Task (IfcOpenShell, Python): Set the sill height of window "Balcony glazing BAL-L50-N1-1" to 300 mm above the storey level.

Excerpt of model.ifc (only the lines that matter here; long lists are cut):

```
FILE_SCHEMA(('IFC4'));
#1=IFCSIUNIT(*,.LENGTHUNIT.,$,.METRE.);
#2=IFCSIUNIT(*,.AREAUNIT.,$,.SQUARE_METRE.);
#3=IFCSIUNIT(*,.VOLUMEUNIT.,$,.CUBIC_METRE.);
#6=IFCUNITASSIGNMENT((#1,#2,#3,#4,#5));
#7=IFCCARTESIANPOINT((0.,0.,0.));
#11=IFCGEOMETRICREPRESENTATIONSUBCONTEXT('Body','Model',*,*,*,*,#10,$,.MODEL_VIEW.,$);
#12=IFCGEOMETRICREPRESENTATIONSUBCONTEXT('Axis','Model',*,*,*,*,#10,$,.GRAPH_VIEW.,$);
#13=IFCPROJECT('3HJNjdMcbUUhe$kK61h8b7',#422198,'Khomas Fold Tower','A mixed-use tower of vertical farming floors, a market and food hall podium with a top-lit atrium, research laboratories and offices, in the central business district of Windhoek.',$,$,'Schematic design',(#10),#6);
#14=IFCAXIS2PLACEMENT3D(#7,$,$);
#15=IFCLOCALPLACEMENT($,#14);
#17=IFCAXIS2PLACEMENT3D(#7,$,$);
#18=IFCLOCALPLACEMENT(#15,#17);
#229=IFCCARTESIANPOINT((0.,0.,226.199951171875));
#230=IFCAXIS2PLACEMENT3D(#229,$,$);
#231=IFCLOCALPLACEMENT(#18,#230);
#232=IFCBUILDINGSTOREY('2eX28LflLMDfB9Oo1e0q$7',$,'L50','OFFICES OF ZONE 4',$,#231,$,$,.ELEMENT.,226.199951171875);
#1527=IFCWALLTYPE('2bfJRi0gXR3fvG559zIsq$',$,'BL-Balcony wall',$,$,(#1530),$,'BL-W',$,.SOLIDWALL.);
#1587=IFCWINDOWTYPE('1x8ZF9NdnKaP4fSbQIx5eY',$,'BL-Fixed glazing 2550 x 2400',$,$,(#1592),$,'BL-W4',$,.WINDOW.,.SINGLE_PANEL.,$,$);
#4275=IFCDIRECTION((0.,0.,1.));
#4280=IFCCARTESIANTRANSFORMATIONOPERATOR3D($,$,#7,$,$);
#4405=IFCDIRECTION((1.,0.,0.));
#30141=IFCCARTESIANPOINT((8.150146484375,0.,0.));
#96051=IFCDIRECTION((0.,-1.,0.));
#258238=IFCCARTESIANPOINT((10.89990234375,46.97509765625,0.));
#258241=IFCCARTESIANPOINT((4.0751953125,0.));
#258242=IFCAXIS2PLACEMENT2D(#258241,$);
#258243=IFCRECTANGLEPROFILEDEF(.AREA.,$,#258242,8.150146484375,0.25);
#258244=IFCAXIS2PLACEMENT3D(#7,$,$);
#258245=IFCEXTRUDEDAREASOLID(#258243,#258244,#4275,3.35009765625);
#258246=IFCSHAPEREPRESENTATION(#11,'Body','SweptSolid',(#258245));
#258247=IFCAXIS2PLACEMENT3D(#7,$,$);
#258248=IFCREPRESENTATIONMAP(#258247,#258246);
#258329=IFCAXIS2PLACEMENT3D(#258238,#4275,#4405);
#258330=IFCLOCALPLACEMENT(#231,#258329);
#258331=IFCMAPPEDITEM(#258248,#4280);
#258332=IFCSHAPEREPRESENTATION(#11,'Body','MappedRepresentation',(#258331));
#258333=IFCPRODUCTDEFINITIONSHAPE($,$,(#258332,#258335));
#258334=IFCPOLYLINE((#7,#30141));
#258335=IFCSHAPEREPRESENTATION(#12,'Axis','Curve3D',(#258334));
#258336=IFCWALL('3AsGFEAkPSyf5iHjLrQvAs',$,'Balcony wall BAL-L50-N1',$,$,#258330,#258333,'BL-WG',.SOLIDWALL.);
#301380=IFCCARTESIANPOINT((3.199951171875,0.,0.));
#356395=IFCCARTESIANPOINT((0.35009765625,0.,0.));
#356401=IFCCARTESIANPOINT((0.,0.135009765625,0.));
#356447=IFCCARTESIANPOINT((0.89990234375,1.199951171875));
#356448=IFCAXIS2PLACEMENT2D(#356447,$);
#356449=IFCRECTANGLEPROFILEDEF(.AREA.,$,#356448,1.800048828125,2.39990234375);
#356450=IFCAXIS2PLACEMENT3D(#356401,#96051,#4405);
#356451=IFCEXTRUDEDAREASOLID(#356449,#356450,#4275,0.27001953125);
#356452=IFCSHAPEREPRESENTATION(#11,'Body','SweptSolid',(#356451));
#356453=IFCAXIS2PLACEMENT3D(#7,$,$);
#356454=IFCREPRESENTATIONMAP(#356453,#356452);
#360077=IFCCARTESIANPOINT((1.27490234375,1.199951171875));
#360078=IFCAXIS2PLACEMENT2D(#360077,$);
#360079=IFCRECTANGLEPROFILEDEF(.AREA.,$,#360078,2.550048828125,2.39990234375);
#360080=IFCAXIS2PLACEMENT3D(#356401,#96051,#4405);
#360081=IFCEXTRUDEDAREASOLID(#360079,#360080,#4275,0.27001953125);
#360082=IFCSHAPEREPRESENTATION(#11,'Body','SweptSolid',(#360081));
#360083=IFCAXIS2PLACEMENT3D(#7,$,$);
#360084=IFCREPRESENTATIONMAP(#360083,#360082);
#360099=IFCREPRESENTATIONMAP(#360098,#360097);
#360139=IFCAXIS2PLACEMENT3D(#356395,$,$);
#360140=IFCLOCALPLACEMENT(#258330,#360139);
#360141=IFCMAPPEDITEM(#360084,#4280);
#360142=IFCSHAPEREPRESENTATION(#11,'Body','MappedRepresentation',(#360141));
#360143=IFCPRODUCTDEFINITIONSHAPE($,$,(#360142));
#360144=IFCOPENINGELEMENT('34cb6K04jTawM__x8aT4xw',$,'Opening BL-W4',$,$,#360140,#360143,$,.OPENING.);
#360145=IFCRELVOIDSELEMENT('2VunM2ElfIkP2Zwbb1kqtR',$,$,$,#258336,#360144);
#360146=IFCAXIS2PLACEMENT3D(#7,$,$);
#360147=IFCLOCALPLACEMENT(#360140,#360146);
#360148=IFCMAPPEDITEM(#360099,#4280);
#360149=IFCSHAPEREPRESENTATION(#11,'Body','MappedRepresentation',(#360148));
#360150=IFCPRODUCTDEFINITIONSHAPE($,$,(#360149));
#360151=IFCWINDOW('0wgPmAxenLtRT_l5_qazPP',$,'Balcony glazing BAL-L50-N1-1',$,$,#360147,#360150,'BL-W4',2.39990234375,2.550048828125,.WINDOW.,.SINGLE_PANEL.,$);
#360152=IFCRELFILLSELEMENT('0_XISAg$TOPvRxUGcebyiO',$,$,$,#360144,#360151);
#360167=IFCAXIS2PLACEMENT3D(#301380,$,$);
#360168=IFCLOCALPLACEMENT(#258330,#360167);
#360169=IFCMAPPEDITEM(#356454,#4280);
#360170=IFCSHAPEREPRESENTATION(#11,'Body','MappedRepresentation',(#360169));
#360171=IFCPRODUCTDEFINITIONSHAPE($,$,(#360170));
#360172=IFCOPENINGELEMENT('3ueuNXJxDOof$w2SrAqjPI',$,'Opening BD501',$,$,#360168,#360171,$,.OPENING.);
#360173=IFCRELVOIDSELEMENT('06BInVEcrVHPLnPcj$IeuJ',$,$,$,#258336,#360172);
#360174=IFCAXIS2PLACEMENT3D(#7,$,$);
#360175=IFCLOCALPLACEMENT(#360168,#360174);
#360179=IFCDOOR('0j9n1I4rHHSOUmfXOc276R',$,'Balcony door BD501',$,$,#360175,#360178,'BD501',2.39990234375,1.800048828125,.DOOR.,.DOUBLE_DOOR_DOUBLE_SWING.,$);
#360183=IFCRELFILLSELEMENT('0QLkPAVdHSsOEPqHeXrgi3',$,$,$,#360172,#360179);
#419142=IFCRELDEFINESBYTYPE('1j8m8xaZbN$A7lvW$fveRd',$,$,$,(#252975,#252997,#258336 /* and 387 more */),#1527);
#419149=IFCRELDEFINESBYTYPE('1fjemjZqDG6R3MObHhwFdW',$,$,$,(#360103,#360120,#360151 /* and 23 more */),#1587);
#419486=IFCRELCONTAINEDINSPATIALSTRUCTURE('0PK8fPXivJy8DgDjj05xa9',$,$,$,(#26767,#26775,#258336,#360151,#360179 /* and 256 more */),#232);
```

```python
import numpy as np
import ifcopenshell
import ifcopenshell.api.geometry
import ifcopenshell.geom
import ifcopenshell.util.element
import ifcopenshell.util.placement
import ifcopenshell.util.shape
import ifcopenshell.util.unit

model = ifcopenshell.open("model.ifc")
unit_scale = ifcopenshell.util.unit.calculate_unit_scale(model)

window = model.by_guid("0wgPmAxenLtRT_l5_qazPP")
opening = window.FillsVoids[0].RelatingOpeningElement
storey = ifcopenshell.util.element.get_container(window, ifc_class="IfcBuildingStorey")
level = ifcopenshell.util.placement.get_local_placement(storey.ObjectPlacement)[2, 3]

# The opening's origin need not be at the sill, so measure its lowest point.
shape = ifcopenshell.geom.create_shape(ifcopenshell.geom.settings(), opening)
bottom = ifcopenshell.util.shape.get_shape_bottom_elevation(shape, shape.geometry) / unit_scale
dz = level + 0.3 / unit_scale - bottom

shift = np.array([0.0, 0.0, dz])
# The window is placed relative to its opening, so it follows when the opening moves.
matrix = ifcopenshell.util.placement.get_local_placement(opening.ObjectPlacement)
matrix[:3, 3] += shift
ifcopenshell.api.geometry.edit_object_placement(
    model, product=opening, matrix=matrix, is_si=False, should_transform_children=True
)

print(f"moved by {dz * unit_scale:+.3f} m")

model.write("model_v2.ifc")
```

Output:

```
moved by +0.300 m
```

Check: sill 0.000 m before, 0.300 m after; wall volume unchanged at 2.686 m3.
